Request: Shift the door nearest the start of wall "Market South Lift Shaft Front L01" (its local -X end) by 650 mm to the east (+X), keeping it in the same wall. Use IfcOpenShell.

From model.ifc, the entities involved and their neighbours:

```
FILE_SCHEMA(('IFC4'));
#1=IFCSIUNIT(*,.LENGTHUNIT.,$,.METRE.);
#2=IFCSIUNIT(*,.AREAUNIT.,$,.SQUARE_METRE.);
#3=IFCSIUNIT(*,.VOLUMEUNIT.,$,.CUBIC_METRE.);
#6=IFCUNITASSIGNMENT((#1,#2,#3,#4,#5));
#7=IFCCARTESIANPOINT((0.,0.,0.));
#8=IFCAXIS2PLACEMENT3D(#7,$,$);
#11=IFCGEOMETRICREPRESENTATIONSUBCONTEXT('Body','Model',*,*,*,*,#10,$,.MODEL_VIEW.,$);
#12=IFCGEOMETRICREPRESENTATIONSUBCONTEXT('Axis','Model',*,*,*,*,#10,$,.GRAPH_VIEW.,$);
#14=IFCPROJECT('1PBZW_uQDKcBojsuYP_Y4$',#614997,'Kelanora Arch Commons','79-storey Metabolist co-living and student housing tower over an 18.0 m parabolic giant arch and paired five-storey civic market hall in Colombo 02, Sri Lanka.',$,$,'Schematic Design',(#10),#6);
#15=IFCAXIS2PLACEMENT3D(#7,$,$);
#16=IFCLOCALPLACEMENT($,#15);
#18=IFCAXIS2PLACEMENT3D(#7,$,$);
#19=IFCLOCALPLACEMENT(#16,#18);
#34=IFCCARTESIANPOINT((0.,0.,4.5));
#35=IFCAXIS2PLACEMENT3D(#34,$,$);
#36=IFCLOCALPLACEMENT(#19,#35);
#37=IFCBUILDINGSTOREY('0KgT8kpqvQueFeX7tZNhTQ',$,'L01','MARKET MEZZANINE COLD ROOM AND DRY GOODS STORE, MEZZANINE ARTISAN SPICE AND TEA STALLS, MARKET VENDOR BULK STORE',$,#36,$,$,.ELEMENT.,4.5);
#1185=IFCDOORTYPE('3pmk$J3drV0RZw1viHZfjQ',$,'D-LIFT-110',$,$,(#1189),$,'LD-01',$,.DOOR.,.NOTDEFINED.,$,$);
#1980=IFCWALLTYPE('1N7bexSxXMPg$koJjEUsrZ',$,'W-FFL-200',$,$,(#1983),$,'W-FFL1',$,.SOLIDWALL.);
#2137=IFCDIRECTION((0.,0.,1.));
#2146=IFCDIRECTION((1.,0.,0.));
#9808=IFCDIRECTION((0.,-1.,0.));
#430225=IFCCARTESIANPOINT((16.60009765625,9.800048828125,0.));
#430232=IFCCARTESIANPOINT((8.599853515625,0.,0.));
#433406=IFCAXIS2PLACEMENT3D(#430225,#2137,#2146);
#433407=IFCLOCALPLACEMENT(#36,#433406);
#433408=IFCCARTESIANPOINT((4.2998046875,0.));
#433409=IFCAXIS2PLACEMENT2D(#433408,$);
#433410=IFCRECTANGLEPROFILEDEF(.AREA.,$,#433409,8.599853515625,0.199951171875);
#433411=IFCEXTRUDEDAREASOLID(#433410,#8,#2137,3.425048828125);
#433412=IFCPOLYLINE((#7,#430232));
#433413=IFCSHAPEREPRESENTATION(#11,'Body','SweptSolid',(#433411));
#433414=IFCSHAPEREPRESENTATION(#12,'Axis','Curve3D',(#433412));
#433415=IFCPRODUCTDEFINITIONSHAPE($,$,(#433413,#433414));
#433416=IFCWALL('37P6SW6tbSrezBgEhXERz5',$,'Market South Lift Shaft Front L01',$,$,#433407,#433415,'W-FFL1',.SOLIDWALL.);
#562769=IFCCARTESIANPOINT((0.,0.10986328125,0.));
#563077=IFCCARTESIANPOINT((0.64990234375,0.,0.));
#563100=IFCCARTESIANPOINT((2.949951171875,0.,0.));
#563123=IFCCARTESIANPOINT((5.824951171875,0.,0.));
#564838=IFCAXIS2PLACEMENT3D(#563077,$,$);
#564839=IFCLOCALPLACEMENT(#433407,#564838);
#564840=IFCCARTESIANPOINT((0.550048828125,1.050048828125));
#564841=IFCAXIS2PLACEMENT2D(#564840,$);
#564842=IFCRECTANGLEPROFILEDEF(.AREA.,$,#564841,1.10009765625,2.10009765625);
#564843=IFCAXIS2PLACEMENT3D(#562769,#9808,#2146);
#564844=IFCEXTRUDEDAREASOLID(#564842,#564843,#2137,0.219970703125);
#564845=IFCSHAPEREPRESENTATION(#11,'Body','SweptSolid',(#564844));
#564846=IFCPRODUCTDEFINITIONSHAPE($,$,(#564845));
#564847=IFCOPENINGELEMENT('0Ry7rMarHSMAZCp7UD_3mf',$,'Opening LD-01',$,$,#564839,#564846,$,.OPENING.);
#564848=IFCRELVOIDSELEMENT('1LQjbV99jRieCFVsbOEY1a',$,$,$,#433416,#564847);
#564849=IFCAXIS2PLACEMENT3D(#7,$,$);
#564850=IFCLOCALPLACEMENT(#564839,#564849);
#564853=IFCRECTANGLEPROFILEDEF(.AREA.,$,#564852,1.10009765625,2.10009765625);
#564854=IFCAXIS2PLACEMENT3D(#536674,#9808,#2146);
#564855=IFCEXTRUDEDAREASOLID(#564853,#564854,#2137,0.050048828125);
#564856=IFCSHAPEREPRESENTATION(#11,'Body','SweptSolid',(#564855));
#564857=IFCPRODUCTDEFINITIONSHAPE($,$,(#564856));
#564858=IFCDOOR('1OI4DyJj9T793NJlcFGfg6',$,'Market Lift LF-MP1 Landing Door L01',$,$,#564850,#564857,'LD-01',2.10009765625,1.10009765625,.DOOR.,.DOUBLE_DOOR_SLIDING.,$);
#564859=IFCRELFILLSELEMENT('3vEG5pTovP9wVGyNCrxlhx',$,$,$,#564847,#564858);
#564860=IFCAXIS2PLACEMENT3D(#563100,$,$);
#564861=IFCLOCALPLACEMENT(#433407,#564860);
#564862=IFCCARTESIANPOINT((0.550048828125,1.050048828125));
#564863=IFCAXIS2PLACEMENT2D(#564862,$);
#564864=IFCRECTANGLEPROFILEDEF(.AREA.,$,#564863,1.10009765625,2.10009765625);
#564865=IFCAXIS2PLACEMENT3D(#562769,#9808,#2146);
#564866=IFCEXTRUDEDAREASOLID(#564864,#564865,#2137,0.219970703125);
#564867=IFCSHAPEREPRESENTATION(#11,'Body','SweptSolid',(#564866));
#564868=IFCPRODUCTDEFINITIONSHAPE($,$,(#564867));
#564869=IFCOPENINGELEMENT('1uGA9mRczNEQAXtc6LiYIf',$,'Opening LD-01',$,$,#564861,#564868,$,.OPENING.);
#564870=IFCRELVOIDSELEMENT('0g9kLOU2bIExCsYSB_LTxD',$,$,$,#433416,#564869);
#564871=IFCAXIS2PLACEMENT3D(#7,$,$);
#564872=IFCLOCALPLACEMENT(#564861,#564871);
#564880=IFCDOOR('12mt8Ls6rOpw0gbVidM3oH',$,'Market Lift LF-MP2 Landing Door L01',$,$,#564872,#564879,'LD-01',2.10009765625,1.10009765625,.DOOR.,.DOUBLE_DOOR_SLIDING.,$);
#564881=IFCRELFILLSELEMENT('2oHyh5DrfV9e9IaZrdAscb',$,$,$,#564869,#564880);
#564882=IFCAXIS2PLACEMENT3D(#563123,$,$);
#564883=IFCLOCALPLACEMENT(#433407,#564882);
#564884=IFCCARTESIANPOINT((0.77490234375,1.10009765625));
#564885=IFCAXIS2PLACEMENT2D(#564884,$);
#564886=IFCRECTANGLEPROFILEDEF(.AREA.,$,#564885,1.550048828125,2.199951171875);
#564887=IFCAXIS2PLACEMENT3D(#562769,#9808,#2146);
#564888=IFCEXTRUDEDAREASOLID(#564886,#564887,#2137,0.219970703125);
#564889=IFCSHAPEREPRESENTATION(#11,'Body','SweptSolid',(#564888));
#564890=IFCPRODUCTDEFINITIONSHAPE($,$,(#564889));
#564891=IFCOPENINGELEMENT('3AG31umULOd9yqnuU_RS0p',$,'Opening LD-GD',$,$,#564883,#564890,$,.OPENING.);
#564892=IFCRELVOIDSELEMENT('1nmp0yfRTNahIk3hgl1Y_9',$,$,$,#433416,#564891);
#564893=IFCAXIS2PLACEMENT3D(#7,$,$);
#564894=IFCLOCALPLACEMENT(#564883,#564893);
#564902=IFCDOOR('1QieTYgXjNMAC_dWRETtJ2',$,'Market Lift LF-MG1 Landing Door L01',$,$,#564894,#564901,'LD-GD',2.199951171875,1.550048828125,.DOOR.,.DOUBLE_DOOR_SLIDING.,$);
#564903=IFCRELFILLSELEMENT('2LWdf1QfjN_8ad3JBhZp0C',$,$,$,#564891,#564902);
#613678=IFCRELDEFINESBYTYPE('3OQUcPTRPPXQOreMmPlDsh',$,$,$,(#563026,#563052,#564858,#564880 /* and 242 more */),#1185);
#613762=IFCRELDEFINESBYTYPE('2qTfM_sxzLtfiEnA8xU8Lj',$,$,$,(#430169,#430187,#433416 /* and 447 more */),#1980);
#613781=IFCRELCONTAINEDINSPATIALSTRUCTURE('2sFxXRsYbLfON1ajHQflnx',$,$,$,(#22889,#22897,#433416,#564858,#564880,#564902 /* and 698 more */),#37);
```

```python
import ifcopenshell
import ifcopenshell.api.geometry
import ifcopenshell.util.placement
import ifcopenshell.util.unit

model = ifcopenshell.open("model.ifc")
unit_scale = ifcopenshell.util.unit.calculate_unit_scale(model)

door = model.by_guid("1OI4DyJj9T793NJlcFGfg6")
opening = door.FillsVoids[0].RelatingOpeningElement
wall = opening.VoidsElements[0].RelatingBuildingElement

wall_matrix = ifcopenshell.util.placement.get_local_placement(wall.ObjectPlacement)
shift = wall_matrix[:3, 0] * 0.65 / unit_scale
before = ifcopenshell.util.placement.get_local_placement(door.ObjectPlacement)[:3, 3].copy()

# The door is placed relative to its opening, so it follows when the opening moves.
matrix = ifcopenshell.util.placement.get_local_placement(opening.ObjectPlacement)
matrix[:3, 3] += shift
ifcopenshell.api.geometry.edit_object_placement(
    model, product=opening, matrix=matrix, is_si=False, should_transform_children=True
)

after = ifcopenshell.util.placement.get_local_placement(door.ObjectPlacement)[:3, 3]
print("door moved by", (after - before).round(3) + 0.0)

model.write("model-out.ifc")
```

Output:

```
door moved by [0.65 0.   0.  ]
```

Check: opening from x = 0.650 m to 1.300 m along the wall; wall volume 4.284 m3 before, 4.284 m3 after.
